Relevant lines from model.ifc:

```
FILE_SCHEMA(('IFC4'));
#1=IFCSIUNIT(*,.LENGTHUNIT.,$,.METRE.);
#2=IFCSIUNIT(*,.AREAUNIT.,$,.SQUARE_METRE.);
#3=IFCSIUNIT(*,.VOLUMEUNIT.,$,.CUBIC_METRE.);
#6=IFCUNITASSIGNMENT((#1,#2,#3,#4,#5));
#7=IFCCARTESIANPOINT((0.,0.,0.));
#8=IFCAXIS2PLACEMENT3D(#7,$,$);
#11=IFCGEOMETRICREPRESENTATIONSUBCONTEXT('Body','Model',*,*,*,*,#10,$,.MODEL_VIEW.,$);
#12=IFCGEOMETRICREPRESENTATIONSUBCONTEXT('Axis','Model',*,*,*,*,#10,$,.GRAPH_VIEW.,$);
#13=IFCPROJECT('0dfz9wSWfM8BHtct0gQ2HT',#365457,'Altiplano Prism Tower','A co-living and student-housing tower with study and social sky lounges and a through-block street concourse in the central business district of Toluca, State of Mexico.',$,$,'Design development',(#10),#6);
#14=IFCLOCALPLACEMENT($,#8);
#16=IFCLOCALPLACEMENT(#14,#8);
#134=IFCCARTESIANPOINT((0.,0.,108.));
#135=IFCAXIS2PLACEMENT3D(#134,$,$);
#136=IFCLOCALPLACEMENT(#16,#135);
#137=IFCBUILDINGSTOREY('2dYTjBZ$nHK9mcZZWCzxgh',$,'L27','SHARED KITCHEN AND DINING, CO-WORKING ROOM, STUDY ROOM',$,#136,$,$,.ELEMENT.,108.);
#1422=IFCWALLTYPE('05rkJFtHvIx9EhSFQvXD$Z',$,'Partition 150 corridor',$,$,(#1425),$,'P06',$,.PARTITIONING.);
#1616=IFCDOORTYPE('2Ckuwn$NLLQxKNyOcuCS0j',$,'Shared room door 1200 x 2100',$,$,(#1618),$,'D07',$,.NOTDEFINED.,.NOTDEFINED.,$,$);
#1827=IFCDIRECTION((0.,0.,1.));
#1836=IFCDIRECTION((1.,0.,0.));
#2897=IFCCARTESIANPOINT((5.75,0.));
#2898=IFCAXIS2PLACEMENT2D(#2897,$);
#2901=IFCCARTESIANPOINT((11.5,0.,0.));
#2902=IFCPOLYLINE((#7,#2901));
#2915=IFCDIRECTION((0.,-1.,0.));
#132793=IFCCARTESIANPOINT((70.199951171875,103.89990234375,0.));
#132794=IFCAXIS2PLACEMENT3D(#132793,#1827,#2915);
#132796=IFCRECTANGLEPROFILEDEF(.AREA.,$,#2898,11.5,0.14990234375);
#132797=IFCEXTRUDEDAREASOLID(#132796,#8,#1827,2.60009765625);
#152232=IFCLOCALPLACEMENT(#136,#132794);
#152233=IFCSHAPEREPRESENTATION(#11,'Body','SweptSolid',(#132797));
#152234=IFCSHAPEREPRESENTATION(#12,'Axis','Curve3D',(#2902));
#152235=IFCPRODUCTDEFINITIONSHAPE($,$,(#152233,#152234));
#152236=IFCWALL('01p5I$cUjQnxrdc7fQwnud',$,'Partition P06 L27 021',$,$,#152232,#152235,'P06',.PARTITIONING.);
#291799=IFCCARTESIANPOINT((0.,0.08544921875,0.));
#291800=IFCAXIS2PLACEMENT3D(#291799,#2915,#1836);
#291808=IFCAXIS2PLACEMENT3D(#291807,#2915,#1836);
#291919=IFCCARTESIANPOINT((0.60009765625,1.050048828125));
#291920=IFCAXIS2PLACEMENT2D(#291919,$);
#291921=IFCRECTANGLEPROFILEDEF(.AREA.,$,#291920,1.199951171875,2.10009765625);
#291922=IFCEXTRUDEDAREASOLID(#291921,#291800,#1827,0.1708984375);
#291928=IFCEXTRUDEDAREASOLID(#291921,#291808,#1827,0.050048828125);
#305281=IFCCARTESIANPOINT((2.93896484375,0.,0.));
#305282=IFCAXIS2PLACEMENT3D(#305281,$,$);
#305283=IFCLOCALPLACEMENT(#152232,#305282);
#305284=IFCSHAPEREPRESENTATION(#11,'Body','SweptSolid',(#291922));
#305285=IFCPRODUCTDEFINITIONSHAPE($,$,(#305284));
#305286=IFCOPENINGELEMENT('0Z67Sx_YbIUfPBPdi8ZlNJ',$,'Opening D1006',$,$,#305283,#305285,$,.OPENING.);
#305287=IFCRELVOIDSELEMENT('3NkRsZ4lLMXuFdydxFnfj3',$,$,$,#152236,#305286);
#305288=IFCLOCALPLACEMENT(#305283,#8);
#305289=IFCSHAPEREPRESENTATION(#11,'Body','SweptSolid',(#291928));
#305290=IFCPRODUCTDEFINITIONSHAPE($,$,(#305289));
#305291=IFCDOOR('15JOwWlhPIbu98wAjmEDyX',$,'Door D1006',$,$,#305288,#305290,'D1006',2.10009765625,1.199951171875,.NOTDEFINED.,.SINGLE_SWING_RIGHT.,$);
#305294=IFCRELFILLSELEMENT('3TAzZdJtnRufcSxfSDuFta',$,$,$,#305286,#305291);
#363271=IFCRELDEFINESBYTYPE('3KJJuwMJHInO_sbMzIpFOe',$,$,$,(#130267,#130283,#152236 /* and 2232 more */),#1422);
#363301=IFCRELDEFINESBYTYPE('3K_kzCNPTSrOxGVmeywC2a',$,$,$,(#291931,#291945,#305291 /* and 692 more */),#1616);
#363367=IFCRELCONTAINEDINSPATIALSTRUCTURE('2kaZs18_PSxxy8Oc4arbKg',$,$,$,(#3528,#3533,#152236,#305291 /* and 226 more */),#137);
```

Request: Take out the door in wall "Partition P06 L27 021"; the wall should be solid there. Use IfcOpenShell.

```python
import ifcopenshell
import ifcopenshell.api.feature
import ifcopenshell.api.root
import ifcopenshell.geom
import ifcopenshell.util.shape

model = ifcopenshell.open("model.ifc")
settings = ifcopenshell.geom.settings()


def volume(element):
    """Net volume in cubic metres, openings subtracted."""
    shape = ifcopenshell.geom.create_shape(settings, element)
    return ifcopenshell.util.shape.get_volume(shape.geometry)


door = model.by_guid("15JOwWlhPIbu98wAjmEDyX")
opening = door.FillsVoids[0].RelatingOpeningElement
wall = opening.VoidsElements[0].RelatingBuildingElement
before = volume(wall)

ifcopenshell.api.root.remove_product(model, product=door)
ifcopenshell.api.feature.remove_feature(model, feature=opening)

after = volume(wall)

print(f"wall volume {before:.3f} -> {after:.3f} m3")

model.write("model_updated.ifc")
```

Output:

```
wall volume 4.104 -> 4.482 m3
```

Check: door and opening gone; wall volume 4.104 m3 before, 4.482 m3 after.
